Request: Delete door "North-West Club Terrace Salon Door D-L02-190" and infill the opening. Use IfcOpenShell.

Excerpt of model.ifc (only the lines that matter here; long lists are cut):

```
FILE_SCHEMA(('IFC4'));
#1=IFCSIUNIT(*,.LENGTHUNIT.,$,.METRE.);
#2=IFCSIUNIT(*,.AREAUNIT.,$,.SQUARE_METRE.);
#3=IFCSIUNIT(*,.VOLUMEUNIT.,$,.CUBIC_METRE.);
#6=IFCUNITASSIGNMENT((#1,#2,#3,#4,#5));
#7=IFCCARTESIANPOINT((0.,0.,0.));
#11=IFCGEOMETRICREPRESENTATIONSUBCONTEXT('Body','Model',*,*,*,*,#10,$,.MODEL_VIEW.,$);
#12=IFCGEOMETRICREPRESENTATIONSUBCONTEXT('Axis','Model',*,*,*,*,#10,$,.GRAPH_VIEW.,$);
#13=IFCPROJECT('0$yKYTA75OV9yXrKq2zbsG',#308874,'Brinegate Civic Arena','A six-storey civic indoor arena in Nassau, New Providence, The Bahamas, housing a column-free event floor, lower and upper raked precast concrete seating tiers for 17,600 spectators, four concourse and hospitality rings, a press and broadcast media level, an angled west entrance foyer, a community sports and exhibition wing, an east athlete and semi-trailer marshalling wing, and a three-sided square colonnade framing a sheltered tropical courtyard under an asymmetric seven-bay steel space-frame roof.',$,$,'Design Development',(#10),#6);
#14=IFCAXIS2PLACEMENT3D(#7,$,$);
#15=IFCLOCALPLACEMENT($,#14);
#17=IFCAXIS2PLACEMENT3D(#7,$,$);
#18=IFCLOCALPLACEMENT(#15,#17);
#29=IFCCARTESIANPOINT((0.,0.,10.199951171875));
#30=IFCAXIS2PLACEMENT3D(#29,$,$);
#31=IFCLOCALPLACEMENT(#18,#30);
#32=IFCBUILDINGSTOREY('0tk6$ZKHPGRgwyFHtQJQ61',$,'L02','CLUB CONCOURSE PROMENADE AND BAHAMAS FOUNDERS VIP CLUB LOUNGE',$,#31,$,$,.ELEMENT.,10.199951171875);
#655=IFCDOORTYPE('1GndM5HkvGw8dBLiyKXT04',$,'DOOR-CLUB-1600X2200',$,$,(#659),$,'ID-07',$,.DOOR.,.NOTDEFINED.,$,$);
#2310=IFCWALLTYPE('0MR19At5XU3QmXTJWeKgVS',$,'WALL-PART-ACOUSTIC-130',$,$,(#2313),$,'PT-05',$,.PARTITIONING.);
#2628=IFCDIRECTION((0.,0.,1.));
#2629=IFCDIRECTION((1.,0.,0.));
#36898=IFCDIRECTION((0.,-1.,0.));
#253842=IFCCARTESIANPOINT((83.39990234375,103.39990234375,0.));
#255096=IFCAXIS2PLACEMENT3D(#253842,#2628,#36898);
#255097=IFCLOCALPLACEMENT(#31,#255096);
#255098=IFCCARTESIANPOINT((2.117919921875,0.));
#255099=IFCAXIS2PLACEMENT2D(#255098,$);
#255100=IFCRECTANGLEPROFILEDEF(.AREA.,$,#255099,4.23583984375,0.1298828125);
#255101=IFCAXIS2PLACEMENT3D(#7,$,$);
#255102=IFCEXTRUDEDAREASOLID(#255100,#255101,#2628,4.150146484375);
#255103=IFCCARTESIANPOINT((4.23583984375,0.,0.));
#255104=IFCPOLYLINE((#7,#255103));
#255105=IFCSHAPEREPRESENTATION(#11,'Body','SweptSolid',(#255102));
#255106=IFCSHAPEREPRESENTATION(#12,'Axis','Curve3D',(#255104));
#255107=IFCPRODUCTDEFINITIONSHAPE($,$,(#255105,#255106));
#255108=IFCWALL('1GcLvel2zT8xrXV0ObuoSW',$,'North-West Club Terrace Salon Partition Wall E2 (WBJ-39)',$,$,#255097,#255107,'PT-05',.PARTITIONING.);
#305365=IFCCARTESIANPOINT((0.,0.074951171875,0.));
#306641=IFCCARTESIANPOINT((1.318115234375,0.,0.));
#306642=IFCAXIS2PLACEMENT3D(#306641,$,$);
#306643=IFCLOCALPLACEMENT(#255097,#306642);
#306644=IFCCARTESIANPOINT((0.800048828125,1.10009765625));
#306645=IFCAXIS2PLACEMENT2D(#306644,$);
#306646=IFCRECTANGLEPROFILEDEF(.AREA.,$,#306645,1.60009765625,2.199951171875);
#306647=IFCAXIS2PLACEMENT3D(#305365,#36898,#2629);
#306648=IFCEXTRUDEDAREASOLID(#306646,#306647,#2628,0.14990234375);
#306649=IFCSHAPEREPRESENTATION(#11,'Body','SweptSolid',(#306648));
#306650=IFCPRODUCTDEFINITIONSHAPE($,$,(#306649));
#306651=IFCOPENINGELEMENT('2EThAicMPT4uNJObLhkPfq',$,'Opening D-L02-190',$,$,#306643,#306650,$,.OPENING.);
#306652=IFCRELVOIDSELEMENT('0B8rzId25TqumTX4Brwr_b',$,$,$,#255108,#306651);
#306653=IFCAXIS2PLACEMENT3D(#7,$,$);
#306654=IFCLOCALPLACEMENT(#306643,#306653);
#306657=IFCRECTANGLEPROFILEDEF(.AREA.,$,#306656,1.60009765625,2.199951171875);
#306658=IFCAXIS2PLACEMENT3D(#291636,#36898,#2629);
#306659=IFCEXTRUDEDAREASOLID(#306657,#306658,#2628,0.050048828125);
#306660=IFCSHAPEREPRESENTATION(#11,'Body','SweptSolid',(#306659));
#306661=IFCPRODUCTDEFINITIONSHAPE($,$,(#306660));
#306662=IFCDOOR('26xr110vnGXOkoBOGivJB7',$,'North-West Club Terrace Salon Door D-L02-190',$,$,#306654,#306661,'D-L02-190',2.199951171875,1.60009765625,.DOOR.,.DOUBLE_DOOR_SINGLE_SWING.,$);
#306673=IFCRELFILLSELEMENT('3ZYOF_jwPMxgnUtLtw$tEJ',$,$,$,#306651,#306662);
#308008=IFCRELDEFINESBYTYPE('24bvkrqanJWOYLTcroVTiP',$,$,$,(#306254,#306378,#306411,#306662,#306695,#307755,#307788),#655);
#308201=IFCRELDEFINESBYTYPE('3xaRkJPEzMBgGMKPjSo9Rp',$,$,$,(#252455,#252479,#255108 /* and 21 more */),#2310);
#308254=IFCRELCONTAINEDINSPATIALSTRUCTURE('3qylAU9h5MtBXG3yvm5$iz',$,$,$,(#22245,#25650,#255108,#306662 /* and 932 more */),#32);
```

```python
import ifcopenshell
import ifcopenshell.api.feature
import ifcopenshell.api.root
import ifcopenshell.geom
import ifcopenshell.util.shape

model = ifcopenshell.open("model.ifc")
settings = ifcopenshell.geom.settings()


def volume(element):
    """Net volume in cubic metres, openings subtracted."""
    shape = ifcopenshell.geom.create_shape(settings, element)
    return ifcopenshell.util.shape.get_volume(shape.geometry)


door = model.by_guid("26xr110vnGXOkoBOGivJB7")
opening = door.FillsVoids[0].RelatingOpeningElement
wall = opening.VoidsElements[0].RelatingBuildingElement
before = volume(wall)

ifcopenshell.api.root.remove_product(model, product=door)
ifcopenshell.api.feature.remove_feature(model, feature=opening)

after = volume(wall)

print(f"wall volume {before:.3f} -> {after:.3f} m3")

model.write("model-out.ifc")
```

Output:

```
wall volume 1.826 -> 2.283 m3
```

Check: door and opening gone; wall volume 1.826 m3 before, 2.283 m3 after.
